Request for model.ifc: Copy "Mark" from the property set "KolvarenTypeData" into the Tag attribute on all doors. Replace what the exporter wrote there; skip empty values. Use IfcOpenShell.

First a look at what the model holds.

```python
import ifcopenshell
import ifcopenshell.util.element

model = ifcopenshell.open("model.ifc")
print(model.schema)
doors = model.by_type("IfcDoor")
print(len(doors), "doors")
for e in doors[:8]:
    source = ifcopenshell.util.element.get_pset(e, "KolvarenTypeData", "Mark")
    target = e.Tag
    print(e.id(), repr(source), repr(target), sep=" | ")
```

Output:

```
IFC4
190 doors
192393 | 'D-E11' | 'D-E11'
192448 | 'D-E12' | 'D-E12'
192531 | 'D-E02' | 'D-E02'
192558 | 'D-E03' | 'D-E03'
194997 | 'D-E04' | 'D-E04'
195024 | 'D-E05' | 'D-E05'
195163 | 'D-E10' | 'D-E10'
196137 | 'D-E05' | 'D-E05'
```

```python
import ifcopenshell
import ifcopenshell.util.element

model = ifcopenshell.open("model.ifc")

count = 0
for e in model.by_type("IfcDoor"):
    value = ifcopenshell.util.element.get_pset(e, "KolvarenTypeData", "Mark")
    current = e.Tag
    if not value or not value.strip() or current == value:
        continue
    e.Tag = value
    count += 1

print(count, "doors updated")

model.write("model_v2.ifc")
```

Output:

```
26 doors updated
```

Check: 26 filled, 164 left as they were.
